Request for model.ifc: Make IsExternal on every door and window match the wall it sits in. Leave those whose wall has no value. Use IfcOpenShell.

First a look at what the model holds.

```python
import ifcopenshell
import ifcopenshell.util.element

model = ifcopenshell.open("model.ifc")
print(model.schema)
seen = {}
for e in model.by_type("IfcDoor") + model.by_type("IfcWindow"):
    if not e.FillsVoids:
        continue
    host = e.FillsVoids[0].RelatingOpeningElement.VoidsElements[0].RelatingBuildingElement
    own = ifcopenshell.util.element.get_pset(e, f"Pset_{e.is_a()[3:].removesuffix('StandardCase')}Common", "IsExternal")
    wall = ifcopenshell.util.element.get_pset(host, "Pset_WallCommon", "IsExternal")
    seen[e.is_a(), own, wall] = seen.get((e.is_a(), own, wall), 0) + 1
for (cls, own, wall), count in sorted(seen.items(), key=str):
    print(count, cls, "IsExternal:", own, "| host wall:", wall)
```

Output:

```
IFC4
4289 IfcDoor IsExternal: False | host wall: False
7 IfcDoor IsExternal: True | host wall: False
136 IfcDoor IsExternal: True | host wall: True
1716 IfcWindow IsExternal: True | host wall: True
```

```python
import ifcopenshell
import ifcopenshell.api.pset
import ifcopenshell.util.element

model = ifcopenshell.open("model.ifc")

count = 0
for ifc_class, pset_name in (("IfcDoor", "Pset_DoorCommon"), ("IfcWindow", "Pset_WindowCommon")):
    for e in model.by_type(ifc_class):
        if not e.FillsVoids:
            continue
        host = e.FillsVoids[0].RelatingOpeningElement.VoidsElements[0].RelatingBuildingElement
        external = ifcopenshell.util.element.get_pset(host, "Pset_WallCommon", "IsExternal")
        if external is None or ifcopenshell.util.element.get_pset(e, pset_name, "IsExternal") == external:
            continue
        pset = ifcopenshell.api.pset.add_pset(model, product=e, name=pset_name)
        ifcopenshell.api.pset.edit_pset(model, pset=pset, properties={"IsExternal": external})
        count += 1

print(count, "updated")

model.write("model_v2.ifc")
```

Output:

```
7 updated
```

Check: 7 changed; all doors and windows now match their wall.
